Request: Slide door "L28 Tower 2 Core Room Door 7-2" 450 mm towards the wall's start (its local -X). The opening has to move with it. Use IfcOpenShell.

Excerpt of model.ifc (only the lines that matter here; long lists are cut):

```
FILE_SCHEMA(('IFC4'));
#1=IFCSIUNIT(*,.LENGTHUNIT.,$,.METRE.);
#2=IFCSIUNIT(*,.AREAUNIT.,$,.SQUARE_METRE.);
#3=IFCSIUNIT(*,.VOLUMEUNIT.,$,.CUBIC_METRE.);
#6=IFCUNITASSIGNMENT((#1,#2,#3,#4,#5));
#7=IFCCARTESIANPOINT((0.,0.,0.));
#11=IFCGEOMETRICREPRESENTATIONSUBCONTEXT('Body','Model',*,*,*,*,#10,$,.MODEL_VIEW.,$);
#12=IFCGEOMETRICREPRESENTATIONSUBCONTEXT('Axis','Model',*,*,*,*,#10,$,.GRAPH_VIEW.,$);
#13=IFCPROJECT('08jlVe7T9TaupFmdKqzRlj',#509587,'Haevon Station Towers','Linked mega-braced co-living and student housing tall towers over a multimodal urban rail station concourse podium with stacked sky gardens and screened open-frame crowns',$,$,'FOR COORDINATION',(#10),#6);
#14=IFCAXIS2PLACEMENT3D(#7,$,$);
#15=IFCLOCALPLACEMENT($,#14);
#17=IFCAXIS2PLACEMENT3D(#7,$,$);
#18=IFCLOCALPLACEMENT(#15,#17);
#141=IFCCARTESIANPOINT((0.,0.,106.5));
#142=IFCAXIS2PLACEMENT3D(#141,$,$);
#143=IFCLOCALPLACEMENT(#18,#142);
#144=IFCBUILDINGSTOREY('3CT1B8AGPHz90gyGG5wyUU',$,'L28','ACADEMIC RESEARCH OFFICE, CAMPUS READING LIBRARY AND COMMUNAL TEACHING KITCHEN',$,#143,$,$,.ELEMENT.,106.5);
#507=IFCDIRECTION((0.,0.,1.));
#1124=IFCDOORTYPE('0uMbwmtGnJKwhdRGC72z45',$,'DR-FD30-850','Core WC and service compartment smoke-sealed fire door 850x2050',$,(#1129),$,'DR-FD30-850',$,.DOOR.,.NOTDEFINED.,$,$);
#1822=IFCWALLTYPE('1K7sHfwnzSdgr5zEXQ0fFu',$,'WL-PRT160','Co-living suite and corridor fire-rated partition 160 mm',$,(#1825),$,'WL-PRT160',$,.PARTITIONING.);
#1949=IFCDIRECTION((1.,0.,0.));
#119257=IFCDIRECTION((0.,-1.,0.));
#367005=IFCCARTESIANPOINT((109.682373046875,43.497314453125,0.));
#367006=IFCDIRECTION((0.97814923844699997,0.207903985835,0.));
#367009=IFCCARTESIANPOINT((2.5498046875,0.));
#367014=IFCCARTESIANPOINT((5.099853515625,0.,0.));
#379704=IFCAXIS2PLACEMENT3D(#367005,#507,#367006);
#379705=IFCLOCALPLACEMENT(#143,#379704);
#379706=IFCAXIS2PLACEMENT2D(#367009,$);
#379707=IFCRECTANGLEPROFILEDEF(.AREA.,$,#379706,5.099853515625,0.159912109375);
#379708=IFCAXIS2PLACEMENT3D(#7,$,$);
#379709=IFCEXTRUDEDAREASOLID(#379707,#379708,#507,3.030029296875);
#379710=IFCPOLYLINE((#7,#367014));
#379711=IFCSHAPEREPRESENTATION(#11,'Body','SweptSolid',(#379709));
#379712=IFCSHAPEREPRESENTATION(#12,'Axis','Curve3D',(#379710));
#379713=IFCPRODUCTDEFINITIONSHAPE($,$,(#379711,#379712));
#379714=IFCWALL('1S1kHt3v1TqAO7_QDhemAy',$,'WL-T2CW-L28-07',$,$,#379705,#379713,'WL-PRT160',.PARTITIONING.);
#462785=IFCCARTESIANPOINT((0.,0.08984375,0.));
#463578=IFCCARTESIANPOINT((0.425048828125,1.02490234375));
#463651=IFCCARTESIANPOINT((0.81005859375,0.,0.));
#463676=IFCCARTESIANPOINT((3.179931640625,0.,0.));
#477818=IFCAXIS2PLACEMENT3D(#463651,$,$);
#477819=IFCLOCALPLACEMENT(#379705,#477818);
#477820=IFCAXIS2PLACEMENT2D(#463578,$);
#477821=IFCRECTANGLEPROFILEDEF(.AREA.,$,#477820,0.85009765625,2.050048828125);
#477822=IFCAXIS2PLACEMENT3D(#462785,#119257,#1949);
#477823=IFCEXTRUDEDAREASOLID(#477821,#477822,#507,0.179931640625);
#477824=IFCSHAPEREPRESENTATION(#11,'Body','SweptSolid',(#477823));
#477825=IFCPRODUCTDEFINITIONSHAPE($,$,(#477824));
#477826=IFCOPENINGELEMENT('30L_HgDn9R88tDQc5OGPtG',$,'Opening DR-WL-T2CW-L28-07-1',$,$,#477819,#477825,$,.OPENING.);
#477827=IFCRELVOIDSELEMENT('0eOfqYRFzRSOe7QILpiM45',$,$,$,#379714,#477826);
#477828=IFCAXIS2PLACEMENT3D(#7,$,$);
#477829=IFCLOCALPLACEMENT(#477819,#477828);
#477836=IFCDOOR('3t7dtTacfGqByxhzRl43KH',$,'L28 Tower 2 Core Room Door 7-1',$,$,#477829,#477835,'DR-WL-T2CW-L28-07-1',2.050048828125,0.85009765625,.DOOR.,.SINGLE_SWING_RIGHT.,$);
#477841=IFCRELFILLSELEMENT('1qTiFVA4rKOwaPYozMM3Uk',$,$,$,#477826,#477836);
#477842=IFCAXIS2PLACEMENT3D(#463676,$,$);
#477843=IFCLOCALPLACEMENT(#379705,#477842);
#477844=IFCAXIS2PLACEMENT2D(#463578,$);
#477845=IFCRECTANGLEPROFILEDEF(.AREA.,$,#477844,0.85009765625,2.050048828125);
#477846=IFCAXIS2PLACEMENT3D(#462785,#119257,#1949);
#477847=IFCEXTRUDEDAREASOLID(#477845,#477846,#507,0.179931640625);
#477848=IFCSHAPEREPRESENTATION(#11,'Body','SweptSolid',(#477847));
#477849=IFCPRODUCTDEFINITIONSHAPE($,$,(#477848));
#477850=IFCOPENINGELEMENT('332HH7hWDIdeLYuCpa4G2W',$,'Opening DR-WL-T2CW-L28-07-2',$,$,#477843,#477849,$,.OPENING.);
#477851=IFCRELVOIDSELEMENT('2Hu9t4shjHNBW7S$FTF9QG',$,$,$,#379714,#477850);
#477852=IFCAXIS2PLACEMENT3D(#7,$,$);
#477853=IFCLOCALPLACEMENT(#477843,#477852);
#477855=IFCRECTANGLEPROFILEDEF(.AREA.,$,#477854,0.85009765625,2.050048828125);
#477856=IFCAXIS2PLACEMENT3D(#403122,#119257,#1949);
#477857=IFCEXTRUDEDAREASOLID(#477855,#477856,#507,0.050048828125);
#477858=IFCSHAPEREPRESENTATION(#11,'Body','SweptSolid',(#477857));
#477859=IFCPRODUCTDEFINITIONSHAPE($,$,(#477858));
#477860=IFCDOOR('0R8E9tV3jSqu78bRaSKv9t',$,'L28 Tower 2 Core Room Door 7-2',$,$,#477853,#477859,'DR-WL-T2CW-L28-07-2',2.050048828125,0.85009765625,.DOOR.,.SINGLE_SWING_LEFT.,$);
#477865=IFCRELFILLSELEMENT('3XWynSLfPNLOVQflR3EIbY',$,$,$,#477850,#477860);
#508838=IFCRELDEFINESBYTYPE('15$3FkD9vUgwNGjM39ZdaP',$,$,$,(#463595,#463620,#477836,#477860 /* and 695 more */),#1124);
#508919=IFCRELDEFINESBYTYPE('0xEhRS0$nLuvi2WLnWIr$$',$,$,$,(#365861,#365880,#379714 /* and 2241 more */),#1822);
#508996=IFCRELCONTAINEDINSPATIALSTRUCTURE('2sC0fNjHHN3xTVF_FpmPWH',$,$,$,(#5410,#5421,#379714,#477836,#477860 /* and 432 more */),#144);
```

```python
import ifcopenshell
import ifcopenshell.api.geometry
import ifcopenshell.util.placement
import ifcopenshell.util.unit

model = ifcopenshell.open("model.ifc")
unit_scale = ifcopenshell.util.unit.calculate_unit_scale(model)

door = model.by_guid("0R8E9tV3jSqu78bRaSKv9t")
opening = door.FillsVoids[0].RelatingOpeningElement
wall = opening.VoidsElements[0].RelatingBuildingElement

wall_matrix = ifcopenshell.util.placement.get_local_placement(wall.ObjectPlacement)
shift = wall_matrix[:3, 0] * -0.45 / unit_scale
before = ifcopenshell.util.placement.get_local_placement(door.ObjectPlacement)[:3, 3].copy()

# The door is placed relative to its opening, so it follows when the opening moves.
matrix = ifcopenshell.util.placement.get_local_placement(opening.ObjectPlacement)
matrix[:3, 3] += shift
ifcopenshell.api.geometry.edit_object_placement(
    model, product=opening, matrix=matrix, is_si=False, should_transform_children=True
)

after = ifcopenshell.util.placement.get_local_placement(door.ObjectPlacement)[:3, 3]
print("door moved by", (after - before).round(3) + 0.0)

model.write("model_edited.ifc")
```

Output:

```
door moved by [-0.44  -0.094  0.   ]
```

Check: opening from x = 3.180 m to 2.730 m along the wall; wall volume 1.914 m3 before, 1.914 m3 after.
